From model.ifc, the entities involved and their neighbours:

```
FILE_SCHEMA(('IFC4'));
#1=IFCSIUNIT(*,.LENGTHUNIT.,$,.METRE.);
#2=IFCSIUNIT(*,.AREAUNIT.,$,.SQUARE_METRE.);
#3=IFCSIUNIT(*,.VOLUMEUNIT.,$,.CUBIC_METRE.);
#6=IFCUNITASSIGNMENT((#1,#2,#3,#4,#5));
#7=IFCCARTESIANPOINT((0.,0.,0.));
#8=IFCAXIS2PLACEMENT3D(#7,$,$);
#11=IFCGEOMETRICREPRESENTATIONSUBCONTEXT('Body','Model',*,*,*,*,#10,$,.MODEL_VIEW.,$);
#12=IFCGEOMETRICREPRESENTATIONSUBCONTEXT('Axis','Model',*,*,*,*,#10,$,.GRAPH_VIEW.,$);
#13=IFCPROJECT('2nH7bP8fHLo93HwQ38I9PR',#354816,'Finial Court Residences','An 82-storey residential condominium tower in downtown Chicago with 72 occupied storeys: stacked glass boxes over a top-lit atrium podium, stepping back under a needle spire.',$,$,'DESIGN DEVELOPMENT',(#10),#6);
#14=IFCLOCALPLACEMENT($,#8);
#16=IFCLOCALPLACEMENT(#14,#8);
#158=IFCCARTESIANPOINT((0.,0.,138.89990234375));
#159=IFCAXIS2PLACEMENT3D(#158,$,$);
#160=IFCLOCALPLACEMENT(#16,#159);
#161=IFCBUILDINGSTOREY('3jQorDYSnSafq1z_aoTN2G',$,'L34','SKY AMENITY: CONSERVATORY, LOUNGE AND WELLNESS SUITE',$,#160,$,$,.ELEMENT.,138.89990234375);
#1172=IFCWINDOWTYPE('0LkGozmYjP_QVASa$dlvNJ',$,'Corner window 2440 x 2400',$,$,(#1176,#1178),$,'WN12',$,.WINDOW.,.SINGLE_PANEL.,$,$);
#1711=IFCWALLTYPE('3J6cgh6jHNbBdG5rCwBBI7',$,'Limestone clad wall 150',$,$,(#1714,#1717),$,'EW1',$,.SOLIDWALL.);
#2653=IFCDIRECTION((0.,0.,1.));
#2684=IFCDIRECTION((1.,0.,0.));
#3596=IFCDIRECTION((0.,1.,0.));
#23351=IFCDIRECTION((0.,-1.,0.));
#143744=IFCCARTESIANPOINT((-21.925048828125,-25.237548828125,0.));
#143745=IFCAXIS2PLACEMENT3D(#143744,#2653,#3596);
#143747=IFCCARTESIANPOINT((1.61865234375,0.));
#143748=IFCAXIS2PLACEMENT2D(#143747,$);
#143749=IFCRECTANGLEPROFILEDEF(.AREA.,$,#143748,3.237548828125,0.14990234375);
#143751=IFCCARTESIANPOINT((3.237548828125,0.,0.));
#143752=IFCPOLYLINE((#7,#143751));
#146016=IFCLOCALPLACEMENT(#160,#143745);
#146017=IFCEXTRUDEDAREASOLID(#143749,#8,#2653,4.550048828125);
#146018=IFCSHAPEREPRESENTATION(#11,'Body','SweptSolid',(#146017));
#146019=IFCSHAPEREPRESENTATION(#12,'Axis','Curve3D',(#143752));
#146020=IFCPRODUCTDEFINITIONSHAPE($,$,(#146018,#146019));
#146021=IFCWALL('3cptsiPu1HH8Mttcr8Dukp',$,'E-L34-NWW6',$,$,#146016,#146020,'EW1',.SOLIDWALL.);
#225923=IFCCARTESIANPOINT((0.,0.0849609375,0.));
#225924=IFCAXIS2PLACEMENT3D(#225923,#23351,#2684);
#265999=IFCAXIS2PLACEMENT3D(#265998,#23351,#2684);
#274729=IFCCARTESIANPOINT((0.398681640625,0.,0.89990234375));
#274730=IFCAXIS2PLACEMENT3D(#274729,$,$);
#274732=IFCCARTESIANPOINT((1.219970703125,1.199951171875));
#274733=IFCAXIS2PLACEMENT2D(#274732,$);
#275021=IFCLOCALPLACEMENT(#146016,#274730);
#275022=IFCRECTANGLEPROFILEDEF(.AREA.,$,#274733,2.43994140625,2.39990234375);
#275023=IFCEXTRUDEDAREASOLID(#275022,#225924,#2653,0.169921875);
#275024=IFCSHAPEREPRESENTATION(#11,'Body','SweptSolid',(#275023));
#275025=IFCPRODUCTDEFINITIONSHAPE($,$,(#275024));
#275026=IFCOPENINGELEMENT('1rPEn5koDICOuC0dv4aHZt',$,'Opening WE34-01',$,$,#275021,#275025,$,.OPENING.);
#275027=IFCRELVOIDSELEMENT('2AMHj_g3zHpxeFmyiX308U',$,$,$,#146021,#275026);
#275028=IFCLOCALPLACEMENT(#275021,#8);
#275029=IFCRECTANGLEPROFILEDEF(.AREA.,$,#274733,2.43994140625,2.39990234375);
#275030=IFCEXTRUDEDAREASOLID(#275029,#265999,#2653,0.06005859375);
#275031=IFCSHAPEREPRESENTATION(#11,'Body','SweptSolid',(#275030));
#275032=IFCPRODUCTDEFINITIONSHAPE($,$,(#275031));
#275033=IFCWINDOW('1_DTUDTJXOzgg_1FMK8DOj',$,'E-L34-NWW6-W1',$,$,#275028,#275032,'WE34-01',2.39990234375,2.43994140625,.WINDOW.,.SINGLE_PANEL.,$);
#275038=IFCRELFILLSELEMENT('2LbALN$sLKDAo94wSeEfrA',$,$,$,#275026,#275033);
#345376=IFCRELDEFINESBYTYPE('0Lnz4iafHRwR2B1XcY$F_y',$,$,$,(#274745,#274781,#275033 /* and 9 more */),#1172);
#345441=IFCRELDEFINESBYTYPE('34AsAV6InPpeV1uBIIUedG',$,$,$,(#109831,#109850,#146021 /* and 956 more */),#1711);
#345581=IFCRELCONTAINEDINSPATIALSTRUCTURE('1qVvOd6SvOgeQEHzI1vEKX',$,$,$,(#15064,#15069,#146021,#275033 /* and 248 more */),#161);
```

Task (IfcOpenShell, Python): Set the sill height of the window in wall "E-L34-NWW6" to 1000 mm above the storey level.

```python
import numpy as np
import ifcopenshell
import ifcopenshell.api.geometry
import ifcopenshell.geom
import ifcopenshell.util.element
import ifcopenshell.util.placement
import ifcopenshell.util.shape
import ifcopenshell.util.unit

model = ifcopenshell.open("model.ifc")
unit_scale = ifcopenshell.util.unit.calculate_unit_scale(model)

window = model.by_guid("1_DTUDTJXOzgg_1FMK8DOj")
opening = window.FillsVoids[0].RelatingOpeningElement
storey = ifcopenshell.util.element.get_container(window, ifc_class="IfcBuildingStorey")
level = ifcopenshell.util.placement.get_local_placement(storey.ObjectPlacement)[2, 3]

# The opening's origin need not be at the sill, so measure its lowest point.
shape = ifcopenshell.geom.create_shape(ifcopenshell.geom.settings(), opening)
bottom = ifcopenshell.util.shape.get_shape_bottom_elevation(shape, shape.geometry) / unit_scale
dz = level + 1 / unit_scale - bottom

shift = np.array([0.0, 0.0, dz])
# The window is placed relative to its opening, so it follows when the opening moves.
matrix = ifcopenshell.util.placement.get_local_placement(opening.ObjectPlacement)
matrix[:3, 3] += shift
ifcopenshell.api.geometry.edit_object_placement(
    model, product=opening, matrix=matrix, is_si=False, should_transform_children=True
)

print(f"moved by {dz * unit_scale:+.3f} m")

model.write("model_v2.ifc")
```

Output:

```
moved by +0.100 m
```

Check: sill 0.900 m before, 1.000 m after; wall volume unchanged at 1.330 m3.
